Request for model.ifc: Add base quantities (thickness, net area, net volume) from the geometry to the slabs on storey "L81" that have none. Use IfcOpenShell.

First a look at what the model holds.

```python
import ifcopenshell
import ifcopenshell.util.element
import ifcopenshell.util.unit

model = ifcopenshell.open("model.ifc")
print(model.schema)
for unit_type in ("LENGTHUNIT", "AREAUNIT", "VOLUMEUNIT"):
    print(unit_type, ifcopenshell.util.unit.calculate_unit_scale(model, unit_type))
storey = next(s for s in model.by_type("IfcBuildingStorey") if s.Name == "L81")
slabs = [e for e in ifcopenshell.util.element.get_decomposition(storey) if e.is_a("IfcSlab")]
for e in sorted(slabs, key=lambda e: e.id()):
    print(e.id(), e.is_a(), e.Name, list(ifcopenshell.util.element.get_psets(e, qtos_only=True)), sep=" | ")
```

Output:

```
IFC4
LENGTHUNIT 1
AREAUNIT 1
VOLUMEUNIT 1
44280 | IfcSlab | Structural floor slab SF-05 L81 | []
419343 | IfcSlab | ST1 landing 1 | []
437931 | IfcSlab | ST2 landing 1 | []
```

```python
import ifcopenshell
import ifcopenshell.api.pset
import ifcopenshell.geom
import ifcopenshell.util.element
import ifcopenshell.util.shape
import ifcopenshell.util.unit

model = ifcopenshell.open("model.ifc")
unit_scale = ifcopenshell.util.unit.calculate_unit_scale(model)
area_scale = ifcopenshell.util.unit.calculate_unit_scale(model, "AREAUNIT")
volume_scale = ifcopenshell.util.unit.calculate_unit_scale(model, "VOLUMEUNIT")
settings = ifcopenshell.geom.settings()

storey = next(s for s in model.by_type("IfcBuildingStorey") if s.Name == "L81")
slabs = [e for e in ifcopenshell.util.element.get_decomposition(storey) if e.is_a("IfcSlab")]

for e in sorted(slabs, key=lambda e: e.id()):
    if ifcopenshell.util.element.get_psets(e, qtos_only=True, should_inherit=False):
        continue
    # Geometry comes back in metres, in the element's own axes.
    shape = ifcopenshell.geom.create_shape(settings, e)
    values = {
        "Width": ifcopenshell.util.shape.get_z(shape.geometry) / unit_scale,
        "NetArea": ifcopenshell.util.shape.get_footprint_area(shape.geometry) / area_scale,
        "NetVolume": ifcopenshell.util.shape.get_volume(shape.geometry) / volume_scale,
    }
    qto = ifcopenshell.api.pset.add_qto(model, product=e, name="Qto_SlabBaseQuantities")
    ifcopenshell.api.pset.edit_qto(model, qto=qto, properties=values)
    print(e.id(), {k: round(v, 3) for k, v in values.items()})

model.write("model_v2.ifc")
```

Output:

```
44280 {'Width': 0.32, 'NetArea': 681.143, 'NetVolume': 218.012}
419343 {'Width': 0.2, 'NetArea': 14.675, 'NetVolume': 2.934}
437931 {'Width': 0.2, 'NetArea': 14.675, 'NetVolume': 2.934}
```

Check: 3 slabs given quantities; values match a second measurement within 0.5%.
